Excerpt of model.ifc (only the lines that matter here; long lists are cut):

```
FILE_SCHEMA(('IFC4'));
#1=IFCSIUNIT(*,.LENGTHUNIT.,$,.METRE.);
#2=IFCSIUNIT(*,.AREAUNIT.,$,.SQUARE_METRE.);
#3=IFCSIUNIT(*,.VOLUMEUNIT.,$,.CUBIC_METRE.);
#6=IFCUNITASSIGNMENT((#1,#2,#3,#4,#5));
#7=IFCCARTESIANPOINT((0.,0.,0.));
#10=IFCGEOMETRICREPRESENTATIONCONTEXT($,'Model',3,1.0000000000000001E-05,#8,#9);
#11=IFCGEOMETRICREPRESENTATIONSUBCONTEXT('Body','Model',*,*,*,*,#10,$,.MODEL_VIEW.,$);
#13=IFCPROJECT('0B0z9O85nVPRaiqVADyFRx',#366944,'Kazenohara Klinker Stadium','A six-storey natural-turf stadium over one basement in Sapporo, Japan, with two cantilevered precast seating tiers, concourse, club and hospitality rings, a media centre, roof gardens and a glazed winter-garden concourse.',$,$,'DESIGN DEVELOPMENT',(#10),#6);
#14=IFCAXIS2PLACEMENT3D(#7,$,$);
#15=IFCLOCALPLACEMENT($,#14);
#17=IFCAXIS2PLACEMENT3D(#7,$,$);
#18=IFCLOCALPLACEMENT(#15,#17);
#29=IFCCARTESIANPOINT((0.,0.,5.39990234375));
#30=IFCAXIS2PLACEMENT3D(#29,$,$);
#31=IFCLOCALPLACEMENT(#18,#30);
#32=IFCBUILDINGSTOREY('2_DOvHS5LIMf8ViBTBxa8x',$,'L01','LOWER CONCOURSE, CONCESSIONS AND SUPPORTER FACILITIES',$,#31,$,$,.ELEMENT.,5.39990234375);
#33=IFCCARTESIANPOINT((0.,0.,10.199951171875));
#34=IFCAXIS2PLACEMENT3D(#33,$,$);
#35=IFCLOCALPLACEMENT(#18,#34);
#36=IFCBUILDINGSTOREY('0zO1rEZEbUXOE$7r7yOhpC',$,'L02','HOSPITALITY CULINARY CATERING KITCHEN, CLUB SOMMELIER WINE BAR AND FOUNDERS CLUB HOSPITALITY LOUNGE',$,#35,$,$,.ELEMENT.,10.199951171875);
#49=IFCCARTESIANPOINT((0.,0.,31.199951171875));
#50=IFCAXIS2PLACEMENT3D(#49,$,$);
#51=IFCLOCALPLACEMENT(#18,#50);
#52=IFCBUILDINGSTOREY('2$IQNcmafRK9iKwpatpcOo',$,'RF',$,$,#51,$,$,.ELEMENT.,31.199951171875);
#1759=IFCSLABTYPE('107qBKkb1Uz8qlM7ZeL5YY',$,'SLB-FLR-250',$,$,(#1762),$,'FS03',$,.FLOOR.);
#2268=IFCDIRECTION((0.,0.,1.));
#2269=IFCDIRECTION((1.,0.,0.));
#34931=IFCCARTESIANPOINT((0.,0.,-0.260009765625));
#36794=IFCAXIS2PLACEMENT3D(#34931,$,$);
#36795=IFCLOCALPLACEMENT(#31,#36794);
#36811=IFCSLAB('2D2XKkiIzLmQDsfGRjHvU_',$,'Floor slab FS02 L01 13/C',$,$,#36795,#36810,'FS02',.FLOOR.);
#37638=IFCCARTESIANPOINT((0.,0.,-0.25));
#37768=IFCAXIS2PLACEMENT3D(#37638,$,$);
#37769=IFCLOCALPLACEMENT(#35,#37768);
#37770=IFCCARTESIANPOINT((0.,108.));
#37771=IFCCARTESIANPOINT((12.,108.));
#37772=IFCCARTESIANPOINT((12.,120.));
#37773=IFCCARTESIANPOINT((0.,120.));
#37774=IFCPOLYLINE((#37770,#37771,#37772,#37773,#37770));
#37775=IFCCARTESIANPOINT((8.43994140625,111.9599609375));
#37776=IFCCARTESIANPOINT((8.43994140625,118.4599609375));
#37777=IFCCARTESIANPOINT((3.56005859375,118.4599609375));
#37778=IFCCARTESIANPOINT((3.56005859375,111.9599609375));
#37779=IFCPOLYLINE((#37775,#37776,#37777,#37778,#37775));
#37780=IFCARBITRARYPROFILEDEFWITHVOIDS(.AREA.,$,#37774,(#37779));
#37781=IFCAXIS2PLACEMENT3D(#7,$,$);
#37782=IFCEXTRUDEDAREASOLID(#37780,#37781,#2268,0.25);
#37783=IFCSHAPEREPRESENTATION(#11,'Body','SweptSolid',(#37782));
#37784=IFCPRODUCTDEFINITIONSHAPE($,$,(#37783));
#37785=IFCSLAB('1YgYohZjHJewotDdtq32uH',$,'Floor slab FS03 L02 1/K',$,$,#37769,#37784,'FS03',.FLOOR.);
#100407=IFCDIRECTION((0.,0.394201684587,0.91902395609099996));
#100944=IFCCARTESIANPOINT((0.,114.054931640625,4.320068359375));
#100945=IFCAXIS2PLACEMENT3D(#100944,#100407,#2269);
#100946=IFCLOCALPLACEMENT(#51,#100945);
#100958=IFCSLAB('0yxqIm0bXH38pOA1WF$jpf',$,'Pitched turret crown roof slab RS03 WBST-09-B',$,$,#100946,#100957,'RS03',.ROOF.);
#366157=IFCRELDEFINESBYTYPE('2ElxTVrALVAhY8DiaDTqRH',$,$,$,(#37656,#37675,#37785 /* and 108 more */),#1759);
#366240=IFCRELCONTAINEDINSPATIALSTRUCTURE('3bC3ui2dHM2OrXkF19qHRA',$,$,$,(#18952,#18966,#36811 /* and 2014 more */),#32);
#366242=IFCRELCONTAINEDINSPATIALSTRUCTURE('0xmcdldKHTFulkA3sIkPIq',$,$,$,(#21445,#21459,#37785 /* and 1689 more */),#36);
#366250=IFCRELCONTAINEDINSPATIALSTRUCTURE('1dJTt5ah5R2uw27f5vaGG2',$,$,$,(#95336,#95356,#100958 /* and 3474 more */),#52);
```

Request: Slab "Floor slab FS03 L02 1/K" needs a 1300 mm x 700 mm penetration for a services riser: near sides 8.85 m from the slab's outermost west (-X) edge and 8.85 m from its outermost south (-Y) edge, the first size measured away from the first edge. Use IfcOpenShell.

```python
import numpy as np
import ifcopenshell
import ifcopenshell.api.feature
import ifcopenshell.api.geometry
import ifcopenshell.api.root
import ifcopenshell.geom
import ifcopenshell.util.placement
import ifcopenshell.util.representation
import ifcopenshell.util.shape
import ifcopenshell.util.unit

model = ifcopenshell.open("model.ifc")
unit_scale = ifcopenshell.util.unit.calculate_unit_scale(model)
settings = ifcopenshell.geom.settings()


def volume(element):
    """Net volume in cubic metres, openings subtracted."""
    shape = ifcopenshell.geom.create_shape(settings, element)
    return ifcopenshell.util.shape.get_volume(shape.geometry)


slab = model.by_id(37785)
before = volume(slab)

# Extent in the slab's own axes, in metres. The edges named are its -X and -Y sides.
slab_shape = ifcopenshell.geom.create_shape(settings, slab)
vertices = ifcopenshell.util.shape.get_vertices(slab_shape.geometry)
x_min, y_min, bottom = vertices.min(axis=0)
top = vertices[:, 2].max()

opening = ifcopenshell.api.root.create_entity(model, ifc_class="IfcOpeningElement", name="Services riser opening", predefined_type="OPENING")
context = ifcopenshell.util.representation.get_context(model, "Model", "Body", "MODEL_VIEW")
width, depth = 1.3, 0.7
outline = [(0.0, 0.0), (width, 0.0), (width, depth), (0.0, depth), (0.0, 0.0)]
# Overshoot both faces by 50 mm so the cut is clean.
shape = ifcopenshell.api.geometry.add_slab_representation(
    model, context=context, depth=top - bottom + 0.1, polyline=outline
)
ifcopenshell.api.geometry.assign_representation(model, product=opening, representation=shape)

matrix = ifcopenshell.util.placement.get_local_placement(slab.ObjectPlacement)
matrix[:, 3] = matrix @ np.append(np.array([x_min + 8.85, y_min + 8.85, bottom - 0.05]) / unit_scale, 1.0)
ifcopenshell.api.geometry.edit_object_placement(model, product=opening, matrix=matrix, is_si=False)
ifcopenshell.api.feature.add_feature(model, feature=opening, element=slab)

after = volume(slab)

print(f"slab volume {before:.3f} -> {after:.3f} m3")

model.write("model_updated.ifc")
```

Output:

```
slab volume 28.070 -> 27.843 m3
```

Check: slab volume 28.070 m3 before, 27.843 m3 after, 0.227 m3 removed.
